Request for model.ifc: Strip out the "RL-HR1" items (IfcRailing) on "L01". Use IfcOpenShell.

First a look at what the model holds.

```python
import ifcopenshell
import ifcopenshell.util.element

model = ifcopenshell.open("model.ifc")
print(model.schema)
storey = next(s for s in model.by_type("IfcBuildingStorey") if s.Name == "L01")
railings = [e for e in ifcopenshell.util.element.get_decomposition(storey) if e.is_a("IfcRailing")]
seen = {}
for e in railings:
    element_type = ifcopenshell.util.element.get_type(e)
    name = element_type.Name if element_type not in (None, e) else None
    seen[name] = seen.get(name, 0) + 1
for name, count in sorted(seen.items(), key=str):
    print(count, "x", name)
```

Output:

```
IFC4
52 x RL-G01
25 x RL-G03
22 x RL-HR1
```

```python
import ifcopenshell
import ifcopenshell.api.root
import ifcopenshell.util.element

model = ifcopenshell.open("model.ifc")

storey = next(s for s in model.by_type("IfcBuildingStorey") if s.Name == "L01")
railings = [e for e in ifcopenshell.util.element.get_decomposition(storey) if e.is_a("IfcRailing")]
targets = [e for e in railings if (t := ifcopenshell.util.element.get_type(e)) not in (None, e) and t.Name == "RL-HR1"]

for e in targets:
    ifcopenshell.api.root.remove_product(model, product=e)
print(len(targets), "removed")

model.write("model_edited.ifc")
```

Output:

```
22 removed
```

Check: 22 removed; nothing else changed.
